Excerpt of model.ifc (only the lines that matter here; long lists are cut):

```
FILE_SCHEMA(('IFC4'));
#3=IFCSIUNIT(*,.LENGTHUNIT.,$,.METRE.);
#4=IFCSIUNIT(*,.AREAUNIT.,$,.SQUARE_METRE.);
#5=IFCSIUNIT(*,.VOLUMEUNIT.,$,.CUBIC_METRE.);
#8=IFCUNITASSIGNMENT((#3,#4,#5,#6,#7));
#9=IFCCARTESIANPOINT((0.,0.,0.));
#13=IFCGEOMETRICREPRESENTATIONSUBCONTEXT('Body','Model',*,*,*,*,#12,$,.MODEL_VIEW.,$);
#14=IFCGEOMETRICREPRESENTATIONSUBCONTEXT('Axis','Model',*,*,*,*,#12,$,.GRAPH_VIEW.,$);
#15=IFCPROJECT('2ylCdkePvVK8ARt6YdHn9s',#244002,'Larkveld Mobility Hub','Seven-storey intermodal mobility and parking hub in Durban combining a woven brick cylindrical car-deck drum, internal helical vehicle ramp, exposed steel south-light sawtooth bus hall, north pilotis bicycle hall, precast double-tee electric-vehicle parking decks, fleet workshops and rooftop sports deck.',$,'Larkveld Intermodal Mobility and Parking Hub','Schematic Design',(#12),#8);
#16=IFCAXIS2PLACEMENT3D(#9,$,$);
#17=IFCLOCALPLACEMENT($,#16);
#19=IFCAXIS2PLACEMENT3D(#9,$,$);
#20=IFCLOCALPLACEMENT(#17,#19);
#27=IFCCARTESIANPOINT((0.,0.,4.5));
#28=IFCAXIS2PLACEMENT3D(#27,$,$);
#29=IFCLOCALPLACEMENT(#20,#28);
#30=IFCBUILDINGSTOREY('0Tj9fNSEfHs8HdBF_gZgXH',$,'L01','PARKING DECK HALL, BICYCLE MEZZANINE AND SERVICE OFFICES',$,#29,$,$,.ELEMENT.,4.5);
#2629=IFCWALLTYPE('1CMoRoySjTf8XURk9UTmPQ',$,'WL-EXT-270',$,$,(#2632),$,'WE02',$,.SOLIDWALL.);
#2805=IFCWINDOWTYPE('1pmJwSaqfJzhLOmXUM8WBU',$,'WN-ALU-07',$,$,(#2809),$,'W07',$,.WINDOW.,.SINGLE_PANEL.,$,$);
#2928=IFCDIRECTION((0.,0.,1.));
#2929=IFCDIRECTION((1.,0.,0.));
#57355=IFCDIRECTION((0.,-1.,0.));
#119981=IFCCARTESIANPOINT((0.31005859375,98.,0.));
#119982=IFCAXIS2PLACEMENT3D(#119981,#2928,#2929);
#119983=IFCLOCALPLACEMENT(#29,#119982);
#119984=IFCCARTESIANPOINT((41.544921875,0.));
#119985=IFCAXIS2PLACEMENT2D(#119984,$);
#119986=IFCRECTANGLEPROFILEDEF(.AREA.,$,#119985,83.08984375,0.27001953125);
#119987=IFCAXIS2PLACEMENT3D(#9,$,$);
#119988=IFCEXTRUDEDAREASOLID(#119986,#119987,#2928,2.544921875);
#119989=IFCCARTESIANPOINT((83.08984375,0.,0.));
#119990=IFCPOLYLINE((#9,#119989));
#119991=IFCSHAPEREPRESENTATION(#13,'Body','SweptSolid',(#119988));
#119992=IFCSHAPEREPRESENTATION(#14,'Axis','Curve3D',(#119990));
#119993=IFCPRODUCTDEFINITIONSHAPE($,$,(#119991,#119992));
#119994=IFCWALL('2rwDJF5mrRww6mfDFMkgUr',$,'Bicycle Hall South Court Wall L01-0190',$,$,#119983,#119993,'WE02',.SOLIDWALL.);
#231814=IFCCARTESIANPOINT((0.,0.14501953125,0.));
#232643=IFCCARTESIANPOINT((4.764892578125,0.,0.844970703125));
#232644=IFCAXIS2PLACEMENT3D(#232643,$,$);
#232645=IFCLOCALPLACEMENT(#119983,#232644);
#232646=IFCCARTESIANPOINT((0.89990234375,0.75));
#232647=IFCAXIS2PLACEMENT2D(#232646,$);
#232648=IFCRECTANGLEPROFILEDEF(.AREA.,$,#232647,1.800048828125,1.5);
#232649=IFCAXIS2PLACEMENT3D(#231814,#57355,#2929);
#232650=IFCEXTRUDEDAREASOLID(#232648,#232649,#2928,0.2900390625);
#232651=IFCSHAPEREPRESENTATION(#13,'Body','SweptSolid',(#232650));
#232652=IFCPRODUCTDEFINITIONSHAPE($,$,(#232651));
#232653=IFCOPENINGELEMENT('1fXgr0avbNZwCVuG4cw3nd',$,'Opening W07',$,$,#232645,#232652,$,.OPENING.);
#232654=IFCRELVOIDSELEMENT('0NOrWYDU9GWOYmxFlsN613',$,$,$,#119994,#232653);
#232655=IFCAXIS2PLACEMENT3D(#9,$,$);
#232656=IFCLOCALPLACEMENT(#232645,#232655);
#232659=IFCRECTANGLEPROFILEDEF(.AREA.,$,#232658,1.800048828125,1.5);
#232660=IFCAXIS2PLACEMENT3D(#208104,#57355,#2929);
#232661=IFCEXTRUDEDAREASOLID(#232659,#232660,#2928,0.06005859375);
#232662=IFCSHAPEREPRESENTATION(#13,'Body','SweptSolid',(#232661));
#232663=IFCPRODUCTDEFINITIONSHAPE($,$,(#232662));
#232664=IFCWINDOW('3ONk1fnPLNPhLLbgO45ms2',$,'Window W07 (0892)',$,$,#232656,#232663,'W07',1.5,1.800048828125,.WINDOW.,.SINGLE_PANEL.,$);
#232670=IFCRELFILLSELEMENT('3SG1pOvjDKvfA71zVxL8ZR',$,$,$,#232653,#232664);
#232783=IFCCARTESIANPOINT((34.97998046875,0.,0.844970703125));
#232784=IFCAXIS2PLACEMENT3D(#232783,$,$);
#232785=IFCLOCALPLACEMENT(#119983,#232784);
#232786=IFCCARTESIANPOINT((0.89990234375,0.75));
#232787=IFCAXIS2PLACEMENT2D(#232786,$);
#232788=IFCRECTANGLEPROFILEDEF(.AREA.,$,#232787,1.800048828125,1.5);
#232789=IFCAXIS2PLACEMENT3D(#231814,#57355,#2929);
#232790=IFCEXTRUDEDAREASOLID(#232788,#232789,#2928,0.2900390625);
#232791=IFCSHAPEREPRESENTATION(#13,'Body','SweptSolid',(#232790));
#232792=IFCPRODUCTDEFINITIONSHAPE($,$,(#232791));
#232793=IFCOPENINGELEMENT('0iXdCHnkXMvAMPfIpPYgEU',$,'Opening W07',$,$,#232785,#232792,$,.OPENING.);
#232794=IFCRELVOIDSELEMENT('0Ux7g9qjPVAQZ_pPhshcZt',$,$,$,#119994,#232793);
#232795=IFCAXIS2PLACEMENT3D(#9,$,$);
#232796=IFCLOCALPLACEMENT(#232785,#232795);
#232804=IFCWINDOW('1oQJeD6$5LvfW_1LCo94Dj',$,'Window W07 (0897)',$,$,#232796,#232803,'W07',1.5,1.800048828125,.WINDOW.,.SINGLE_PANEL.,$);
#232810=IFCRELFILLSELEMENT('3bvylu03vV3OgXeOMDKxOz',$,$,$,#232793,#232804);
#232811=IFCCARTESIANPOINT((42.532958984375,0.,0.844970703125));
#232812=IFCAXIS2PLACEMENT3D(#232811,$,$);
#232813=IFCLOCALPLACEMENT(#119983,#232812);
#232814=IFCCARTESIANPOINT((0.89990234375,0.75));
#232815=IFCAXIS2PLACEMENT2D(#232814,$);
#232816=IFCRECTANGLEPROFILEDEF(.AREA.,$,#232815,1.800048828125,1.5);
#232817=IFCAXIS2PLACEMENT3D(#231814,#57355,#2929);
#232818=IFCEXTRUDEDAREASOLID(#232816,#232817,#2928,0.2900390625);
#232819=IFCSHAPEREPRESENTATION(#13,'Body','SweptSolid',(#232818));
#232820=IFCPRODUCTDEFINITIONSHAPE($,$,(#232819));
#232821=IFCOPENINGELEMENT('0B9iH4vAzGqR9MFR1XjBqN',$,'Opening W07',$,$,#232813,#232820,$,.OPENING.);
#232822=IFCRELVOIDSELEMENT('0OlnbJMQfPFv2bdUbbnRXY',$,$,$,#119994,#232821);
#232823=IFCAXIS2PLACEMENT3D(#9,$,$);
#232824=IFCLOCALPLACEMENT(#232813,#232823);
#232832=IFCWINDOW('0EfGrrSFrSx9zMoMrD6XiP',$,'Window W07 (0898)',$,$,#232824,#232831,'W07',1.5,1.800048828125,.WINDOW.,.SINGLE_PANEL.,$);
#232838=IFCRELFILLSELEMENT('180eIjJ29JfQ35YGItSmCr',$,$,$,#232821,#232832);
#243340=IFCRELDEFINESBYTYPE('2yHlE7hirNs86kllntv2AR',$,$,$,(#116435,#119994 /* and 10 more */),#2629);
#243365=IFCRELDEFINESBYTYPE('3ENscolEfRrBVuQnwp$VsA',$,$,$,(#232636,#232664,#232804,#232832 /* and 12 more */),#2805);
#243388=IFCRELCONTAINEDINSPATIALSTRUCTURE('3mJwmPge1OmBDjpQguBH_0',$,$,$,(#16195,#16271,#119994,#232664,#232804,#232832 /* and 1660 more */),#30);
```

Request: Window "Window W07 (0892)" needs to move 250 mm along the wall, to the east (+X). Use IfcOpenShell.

```python
import ifcopenshell
import ifcopenshell.api.geometry
import ifcopenshell.util.placement
import ifcopenshell.util.unit

model = ifcopenshell.open("model.ifc")
unit_scale = ifcopenshell.util.unit.calculate_unit_scale(model)

window = model.by_guid("3ONk1fnPLNPhLLbgO45ms2")
opening = window.FillsVoids[0].RelatingOpeningElement
wall = opening.VoidsElements[0].RelatingBuildingElement

wall_matrix = ifcopenshell.util.placement.get_local_placement(wall.ObjectPlacement)
shift = wall_matrix[:3, 0] * 0.25 / unit_scale
before = ifcopenshell.util.placement.get_local_placement(window.ObjectPlacement)[:3, 3].copy()

# The window is placed relative to its opening, so it follows when the opening moves.
matrix = ifcopenshell.util.placement.get_local_placement(opening.ObjectPlacement)
matrix[:3, 3] += shift
ifcopenshell.api.geometry.edit_object_placement(
    model, product=opening, matrix=matrix, is_si=False, should_transform_children=True
)

after = ifcopenshell.util.placement.get_local_placement(window.ObjectPlacement)[:3, 3]
print("window moved by", (after - before).round(3) + 0.0)

model.write("model_updated.ifc")
```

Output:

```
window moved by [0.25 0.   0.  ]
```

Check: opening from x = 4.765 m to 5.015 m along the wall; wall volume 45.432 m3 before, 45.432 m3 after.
